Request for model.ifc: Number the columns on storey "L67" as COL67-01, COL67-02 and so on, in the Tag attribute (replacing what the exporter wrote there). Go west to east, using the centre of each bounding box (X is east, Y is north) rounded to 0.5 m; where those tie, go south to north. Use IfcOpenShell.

First a look at what the model holds.

```python
import ifcopenshell
import ifcopenshell.util.element
import ifcopenshell.util.placement

model = ifcopenshell.open("model.ifc")
print(model.schema)
storey = next(s for s in model.by_type("IfcBuildingStorey") if s.Name == "L67")
columns = [e for e in ifcopenshell.util.element.get_decomposition(storey) if e.is_a("IfcColumn")]
for e in sorted(columns, key=lambda e: e.id()):
    origin = ifcopenshell.util.placement.get_local_placement(e.ObjectPlacement)[:3, 3]
    print(e.id(), e.Tag, e.Name, origin.round(2) + 0.0, sep=" | ")
```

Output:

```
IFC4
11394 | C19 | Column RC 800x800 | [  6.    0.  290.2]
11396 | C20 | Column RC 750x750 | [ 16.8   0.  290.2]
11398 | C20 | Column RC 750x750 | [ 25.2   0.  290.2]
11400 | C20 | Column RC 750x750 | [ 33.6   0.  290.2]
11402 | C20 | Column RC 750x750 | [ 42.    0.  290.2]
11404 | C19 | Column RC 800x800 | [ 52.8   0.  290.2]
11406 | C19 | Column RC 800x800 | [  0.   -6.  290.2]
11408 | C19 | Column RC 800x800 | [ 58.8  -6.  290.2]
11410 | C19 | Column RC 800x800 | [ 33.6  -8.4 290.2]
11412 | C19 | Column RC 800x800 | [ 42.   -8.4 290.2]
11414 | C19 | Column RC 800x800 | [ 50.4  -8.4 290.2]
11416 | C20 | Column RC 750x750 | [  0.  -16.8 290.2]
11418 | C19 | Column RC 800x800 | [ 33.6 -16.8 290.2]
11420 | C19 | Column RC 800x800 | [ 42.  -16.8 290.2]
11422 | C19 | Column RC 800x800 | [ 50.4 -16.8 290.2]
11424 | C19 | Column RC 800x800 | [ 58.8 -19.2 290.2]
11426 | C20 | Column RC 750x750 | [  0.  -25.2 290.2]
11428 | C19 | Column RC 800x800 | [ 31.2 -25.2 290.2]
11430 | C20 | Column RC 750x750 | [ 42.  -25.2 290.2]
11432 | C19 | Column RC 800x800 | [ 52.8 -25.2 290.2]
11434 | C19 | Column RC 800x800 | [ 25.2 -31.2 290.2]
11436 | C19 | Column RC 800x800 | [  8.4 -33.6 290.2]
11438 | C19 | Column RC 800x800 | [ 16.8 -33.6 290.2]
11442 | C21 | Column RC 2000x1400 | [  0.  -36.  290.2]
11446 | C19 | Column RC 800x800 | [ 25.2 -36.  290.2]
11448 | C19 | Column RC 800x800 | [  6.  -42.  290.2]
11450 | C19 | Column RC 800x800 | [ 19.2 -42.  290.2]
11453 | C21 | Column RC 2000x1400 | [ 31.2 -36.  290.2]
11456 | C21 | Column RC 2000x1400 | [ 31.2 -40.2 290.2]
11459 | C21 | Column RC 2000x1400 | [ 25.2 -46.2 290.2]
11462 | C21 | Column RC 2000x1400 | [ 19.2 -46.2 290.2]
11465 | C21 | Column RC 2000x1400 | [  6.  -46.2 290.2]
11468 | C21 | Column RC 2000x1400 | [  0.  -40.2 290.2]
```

```python
import ifcopenshell
import ifcopenshell.geom
import ifcopenshell.util.element
import ifcopenshell.util.shape

model = ifcopenshell.open("model.ifc")
settings = ifcopenshell.geom.settings()
settings.set("use-world-coords", True)


def centre(element):
    shape = ifcopenshell.geom.create_shape(settings, element)
    return ifcopenshell.util.shape.get_bbox_centroid(shape.geometry)


storey = next(s for s in model.by_type("IfcBuildingStorey") if s.Name == "L67")
columns = [e for e in ifcopenshell.util.element.get_decomposition(storey) if e.is_a("IfcColumn")]

# Insertion points can sit at a corner or the storey origin, so sort by the geometry (in metres).
centres = {e: centre(e) for e in columns}
columns.sort(key=lambda e: (round(centres[e][0] / 0.5), centres[e][1]))

for i, e in enumerate(columns, start=1):
    number = f"COL67-{i:02d}"
    e.Tag = number
    print(e.id(), number)

model.write("model_v2.ifc")
```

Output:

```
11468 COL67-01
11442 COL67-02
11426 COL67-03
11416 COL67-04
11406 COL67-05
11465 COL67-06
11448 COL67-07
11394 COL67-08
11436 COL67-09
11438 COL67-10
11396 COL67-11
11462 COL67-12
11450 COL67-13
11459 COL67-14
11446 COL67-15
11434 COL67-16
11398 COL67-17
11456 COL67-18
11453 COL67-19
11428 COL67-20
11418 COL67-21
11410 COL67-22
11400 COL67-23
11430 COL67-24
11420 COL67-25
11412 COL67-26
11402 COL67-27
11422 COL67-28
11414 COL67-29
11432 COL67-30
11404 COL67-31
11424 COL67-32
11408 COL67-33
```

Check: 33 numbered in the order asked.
